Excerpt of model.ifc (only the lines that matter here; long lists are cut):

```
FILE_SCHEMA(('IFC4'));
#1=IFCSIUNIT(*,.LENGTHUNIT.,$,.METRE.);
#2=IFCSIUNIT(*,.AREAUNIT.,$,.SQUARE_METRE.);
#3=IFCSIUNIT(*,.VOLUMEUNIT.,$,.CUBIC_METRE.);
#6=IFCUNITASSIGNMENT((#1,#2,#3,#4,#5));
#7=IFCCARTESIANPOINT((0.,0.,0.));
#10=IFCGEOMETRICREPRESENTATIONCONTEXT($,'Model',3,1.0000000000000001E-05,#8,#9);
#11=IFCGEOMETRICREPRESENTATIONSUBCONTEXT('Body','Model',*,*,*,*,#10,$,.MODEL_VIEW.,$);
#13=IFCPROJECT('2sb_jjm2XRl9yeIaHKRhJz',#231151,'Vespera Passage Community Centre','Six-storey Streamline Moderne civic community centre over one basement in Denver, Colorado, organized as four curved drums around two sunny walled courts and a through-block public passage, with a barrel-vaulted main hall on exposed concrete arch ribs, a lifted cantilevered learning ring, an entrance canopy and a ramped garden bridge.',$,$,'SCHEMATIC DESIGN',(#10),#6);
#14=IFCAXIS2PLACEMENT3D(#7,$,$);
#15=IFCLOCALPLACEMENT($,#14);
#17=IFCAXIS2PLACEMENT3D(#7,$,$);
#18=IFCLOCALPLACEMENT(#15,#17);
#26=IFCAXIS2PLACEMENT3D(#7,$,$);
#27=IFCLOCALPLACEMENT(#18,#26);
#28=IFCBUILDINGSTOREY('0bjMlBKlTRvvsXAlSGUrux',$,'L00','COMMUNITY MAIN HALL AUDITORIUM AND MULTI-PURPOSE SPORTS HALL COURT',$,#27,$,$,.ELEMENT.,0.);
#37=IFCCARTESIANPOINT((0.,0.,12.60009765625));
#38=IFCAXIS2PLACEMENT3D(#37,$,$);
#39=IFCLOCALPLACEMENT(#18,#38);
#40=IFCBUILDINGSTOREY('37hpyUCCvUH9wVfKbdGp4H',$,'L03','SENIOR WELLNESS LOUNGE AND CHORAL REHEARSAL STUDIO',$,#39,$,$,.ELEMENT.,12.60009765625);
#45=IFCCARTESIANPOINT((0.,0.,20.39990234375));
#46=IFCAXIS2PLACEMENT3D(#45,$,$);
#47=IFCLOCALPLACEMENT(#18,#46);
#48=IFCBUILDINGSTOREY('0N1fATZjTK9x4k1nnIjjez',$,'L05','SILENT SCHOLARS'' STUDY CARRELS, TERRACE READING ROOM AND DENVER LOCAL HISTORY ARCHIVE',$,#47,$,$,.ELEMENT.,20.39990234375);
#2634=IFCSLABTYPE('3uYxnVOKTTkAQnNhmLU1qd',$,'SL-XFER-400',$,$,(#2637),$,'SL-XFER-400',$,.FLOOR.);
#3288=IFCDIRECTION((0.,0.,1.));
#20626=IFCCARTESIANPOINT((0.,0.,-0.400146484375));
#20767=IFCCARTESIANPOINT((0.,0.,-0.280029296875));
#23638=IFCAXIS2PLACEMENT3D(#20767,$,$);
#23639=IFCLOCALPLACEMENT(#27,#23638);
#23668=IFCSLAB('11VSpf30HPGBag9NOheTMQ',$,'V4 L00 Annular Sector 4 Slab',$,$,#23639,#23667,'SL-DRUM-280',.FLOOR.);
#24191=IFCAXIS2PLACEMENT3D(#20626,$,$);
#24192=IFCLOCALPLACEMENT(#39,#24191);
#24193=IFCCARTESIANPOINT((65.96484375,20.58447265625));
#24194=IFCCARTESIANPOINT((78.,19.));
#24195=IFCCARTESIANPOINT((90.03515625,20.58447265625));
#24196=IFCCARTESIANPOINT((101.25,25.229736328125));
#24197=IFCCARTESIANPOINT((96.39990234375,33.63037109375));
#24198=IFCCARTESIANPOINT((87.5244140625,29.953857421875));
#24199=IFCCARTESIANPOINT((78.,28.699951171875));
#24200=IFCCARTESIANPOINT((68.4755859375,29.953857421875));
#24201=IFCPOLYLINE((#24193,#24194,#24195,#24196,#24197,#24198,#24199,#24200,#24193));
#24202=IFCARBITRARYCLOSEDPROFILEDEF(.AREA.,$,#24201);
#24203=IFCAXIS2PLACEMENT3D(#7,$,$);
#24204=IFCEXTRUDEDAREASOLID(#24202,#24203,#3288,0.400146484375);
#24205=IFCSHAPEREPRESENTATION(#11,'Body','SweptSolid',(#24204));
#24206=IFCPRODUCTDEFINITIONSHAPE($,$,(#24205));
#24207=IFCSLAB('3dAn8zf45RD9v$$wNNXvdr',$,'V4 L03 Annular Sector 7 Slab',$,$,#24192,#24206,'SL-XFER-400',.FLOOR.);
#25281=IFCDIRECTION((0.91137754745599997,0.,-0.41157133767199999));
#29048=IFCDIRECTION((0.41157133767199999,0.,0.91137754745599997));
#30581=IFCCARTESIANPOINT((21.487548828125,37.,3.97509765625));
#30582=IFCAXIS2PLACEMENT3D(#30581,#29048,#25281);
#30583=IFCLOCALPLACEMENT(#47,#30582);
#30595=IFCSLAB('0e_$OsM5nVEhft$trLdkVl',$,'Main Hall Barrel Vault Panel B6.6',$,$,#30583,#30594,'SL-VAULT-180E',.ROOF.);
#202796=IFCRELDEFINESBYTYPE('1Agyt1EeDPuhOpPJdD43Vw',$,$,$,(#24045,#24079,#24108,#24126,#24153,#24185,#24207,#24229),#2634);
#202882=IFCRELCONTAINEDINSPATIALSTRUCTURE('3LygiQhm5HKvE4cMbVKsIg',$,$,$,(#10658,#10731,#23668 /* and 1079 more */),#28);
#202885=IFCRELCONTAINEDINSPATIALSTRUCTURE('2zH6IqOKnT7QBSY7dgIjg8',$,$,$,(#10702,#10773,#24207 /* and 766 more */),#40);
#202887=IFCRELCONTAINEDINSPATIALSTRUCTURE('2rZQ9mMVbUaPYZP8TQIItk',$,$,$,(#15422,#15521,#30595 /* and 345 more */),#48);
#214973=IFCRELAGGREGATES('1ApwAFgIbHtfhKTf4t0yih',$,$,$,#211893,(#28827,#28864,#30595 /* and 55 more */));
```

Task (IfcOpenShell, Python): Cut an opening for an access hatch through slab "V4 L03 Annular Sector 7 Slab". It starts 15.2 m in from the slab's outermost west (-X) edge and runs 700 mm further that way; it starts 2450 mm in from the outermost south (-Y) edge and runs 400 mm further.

```python
import numpy as np
import ifcopenshell
import ifcopenshell.api.feature
import ifcopenshell.api.geometry
import ifcopenshell.api.root
import ifcopenshell.geom
import ifcopenshell.util.placement
import ifcopenshell.util.representation
import ifcopenshell.util.shape
import ifcopenshell.util.unit

model = ifcopenshell.open("model.ifc")
unit_scale = ifcopenshell.util.unit.calculate_unit_scale(model)
settings = ifcopenshell.geom.settings()


def volume(element):
    """Net volume in cubic metres, openings subtracted."""
    shape = ifcopenshell.geom.create_shape(settings, element)
    return ifcopenshell.util.shape.get_volume(shape.geometry)


slab = model.by_id(24207)
before = volume(slab)

# Extent in the slab's own axes, in metres. The edges named are its -X and -Y sides.
slab_shape = ifcopenshell.geom.create_shape(settings, slab)
vertices = ifcopenshell.util.shape.get_vertices(slab_shape.geometry)
x_min, y_min, bottom = vertices.min(axis=0)
top = vertices[:, 2].max()

opening = ifcopenshell.api.root.create_entity(model, ifc_class="IfcOpeningElement", name="Access hatch opening", predefined_type="OPENING")
context = ifcopenshell.util.representation.get_context(model, "Model", "Body", "MODEL_VIEW")
width, depth = 0.7, 0.4
outline = [(0.0, 0.0), (width, 0.0), (width, depth), (0.0, depth), (0.0, 0.0)]
# Overshoot both faces by 50 mm so the cut is clean.
shape = ifcopenshell.api.geometry.add_slab_representation(
    model, context=context, depth=top - bottom + 0.1, polyline=outline
)
ifcopenshell.api.geometry.assign_representation(model, product=opening, representation=shape)

matrix = ifcopenshell.util.placement.get_local_placement(slab.ObjectPlacement)
matrix[:, 3] = matrix @ np.append(np.array([x_min + 15.2, y_min + 2.45, bottom - 0.05]) / unit_scale, 1.0)
ifcopenshell.api.geometry.edit_object_placement(model, product=opening, matrix=matrix, is_si=False)
ifcopenshell.api.feature.add_feature(model, feature=opening, element=slab)

after = volume(slab)

print(f"slab volume {before:.3f} -> {after:.3f} m3")

model.write("model-out.ifc")
```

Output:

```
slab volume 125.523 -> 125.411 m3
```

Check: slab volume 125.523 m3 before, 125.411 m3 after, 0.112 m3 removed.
